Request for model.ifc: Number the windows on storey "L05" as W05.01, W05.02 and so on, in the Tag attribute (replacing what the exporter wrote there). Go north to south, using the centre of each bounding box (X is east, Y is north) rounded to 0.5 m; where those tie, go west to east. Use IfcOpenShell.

First a look at what the model holds.

```python
import ifcopenshell
import ifcopenshell.util.element
import ifcopenshell.util.placement

model = ifcopenshell.open("model.ifc")
print(model.schema)
storey = next(s for s in model.by_type("IfcBuildingStorey") if s.Name == "L05")
windows = [e for e in ifcopenshell.util.element.get_decomposition(storey) if e.is_a("IfcWindow")]
for e in sorted(windows, key=lambda e: e.id()):
    origin = ifcopenshell.util.placement.get_local_placement(e.ObjectPlacement)[:3, 3]
    print(e.id(), e.Tag, e.Name, origin.round(2) + 0.0, sep=" | ")
```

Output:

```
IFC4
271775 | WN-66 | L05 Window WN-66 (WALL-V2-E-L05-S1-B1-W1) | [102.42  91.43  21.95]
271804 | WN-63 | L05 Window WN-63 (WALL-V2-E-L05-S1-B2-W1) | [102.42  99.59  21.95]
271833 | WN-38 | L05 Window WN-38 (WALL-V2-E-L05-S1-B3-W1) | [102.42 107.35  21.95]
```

```python
import ifcopenshell
import ifcopenshell.geom
import ifcopenshell.util.element
import ifcopenshell.util.shape

model = ifcopenshell.open("model.ifc")
settings = ifcopenshell.geom.settings()
settings.set("use-world-coords", True)


def centre(element):
    shape = ifcopenshell.geom.create_shape(settings, element)
    return ifcopenshell.util.shape.get_bbox_centroid(shape.geometry)


storey = next(s for s in model.by_type("IfcBuildingStorey") if s.Name == "L05")
windows = [e for e in ifcopenshell.util.element.get_decomposition(storey) if e.is_a("IfcWindow")]

# Insertion points can sit at a corner or the storey origin, so sort by the geometry (in metres).
centres = {e: centre(e) for e in windows}
windows.sort(key=lambda e: (-round(centres[e][1] / 0.5), centres[e][0]))

for i, e in enumerate(windows, start=1):
    number = f"W05.{i:02d}"
    e.Tag = number
    print(e.id(), number)

model.write("model_v2.ifc")
```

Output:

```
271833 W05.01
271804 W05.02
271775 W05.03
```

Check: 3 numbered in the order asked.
